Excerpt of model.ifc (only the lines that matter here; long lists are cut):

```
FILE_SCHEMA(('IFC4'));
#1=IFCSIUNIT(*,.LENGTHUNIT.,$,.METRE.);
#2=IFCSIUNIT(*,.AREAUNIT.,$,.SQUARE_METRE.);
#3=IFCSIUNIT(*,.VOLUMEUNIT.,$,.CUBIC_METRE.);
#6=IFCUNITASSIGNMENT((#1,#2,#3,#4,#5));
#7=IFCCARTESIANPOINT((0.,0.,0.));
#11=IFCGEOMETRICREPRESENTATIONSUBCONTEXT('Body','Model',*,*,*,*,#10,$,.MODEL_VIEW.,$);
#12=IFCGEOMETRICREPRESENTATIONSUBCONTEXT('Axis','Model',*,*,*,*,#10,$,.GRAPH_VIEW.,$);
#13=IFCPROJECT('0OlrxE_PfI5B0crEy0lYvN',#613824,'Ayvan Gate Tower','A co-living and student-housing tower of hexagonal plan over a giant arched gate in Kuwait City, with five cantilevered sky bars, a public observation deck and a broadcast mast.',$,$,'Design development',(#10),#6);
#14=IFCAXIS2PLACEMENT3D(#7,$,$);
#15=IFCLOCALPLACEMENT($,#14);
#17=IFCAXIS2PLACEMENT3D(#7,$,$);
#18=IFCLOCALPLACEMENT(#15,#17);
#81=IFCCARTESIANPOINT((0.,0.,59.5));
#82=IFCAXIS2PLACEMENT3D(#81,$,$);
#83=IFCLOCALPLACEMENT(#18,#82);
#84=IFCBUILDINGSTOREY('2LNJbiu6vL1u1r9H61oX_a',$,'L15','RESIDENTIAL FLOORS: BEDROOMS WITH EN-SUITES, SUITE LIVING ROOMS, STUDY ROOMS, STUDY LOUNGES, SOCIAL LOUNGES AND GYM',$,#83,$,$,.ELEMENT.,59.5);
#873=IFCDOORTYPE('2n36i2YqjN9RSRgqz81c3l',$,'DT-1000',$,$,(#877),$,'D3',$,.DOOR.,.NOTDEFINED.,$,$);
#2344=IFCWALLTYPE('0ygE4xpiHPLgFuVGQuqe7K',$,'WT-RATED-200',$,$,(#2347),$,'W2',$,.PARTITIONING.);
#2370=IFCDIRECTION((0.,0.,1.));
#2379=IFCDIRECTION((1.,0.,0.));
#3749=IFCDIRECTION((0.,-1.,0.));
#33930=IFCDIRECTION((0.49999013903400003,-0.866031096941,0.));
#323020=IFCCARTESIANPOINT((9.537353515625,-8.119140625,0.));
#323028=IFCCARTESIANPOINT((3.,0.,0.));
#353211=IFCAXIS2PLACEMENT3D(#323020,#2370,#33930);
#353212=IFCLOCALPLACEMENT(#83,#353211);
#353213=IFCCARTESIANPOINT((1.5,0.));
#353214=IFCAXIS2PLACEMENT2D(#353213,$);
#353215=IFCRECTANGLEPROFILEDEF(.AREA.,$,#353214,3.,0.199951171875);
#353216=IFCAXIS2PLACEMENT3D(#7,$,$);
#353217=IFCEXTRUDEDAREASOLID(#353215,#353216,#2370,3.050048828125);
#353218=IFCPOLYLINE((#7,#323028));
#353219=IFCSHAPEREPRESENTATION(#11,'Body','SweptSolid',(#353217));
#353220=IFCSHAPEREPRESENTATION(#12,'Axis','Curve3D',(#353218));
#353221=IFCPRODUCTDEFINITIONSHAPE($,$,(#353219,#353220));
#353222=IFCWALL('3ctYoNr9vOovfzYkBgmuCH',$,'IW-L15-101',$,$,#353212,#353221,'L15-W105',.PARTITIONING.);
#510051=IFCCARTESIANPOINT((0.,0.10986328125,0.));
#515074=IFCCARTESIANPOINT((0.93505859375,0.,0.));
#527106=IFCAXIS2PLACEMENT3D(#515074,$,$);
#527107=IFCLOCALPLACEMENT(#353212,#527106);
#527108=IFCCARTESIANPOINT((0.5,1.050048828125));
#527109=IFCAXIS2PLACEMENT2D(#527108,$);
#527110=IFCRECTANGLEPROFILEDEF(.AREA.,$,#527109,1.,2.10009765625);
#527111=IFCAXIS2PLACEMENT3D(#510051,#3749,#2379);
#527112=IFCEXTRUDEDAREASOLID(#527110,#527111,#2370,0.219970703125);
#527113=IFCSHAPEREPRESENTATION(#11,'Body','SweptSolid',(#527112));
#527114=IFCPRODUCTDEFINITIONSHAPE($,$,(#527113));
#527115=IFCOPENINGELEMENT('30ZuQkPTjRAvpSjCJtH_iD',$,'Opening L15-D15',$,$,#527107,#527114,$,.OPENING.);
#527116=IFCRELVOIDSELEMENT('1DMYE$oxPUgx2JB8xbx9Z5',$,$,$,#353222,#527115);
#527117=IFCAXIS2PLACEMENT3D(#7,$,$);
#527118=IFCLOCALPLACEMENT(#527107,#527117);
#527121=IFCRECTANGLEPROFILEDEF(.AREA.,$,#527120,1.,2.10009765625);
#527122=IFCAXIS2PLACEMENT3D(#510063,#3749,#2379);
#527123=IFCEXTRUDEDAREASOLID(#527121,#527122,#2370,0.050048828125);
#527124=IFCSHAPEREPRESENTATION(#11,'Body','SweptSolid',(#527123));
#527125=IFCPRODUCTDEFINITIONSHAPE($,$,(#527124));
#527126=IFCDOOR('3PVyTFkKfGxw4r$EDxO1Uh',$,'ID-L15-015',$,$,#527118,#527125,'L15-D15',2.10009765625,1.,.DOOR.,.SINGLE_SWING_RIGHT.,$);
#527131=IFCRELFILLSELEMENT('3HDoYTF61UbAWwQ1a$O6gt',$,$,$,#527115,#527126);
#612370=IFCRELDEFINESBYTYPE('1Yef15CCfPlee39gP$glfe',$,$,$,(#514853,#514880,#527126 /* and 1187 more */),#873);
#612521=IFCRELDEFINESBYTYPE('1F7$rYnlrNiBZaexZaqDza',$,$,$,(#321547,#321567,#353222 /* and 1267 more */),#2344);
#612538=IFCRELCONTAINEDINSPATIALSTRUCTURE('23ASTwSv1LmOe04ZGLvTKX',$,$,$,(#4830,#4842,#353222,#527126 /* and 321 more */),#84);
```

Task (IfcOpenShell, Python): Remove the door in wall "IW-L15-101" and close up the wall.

```python
import ifcopenshell
import ifcopenshell.api.feature
import ifcopenshell.api.root
import ifcopenshell.geom
import ifcopenshell.util.shape

model = ifcopenshell.open("model.ifc")
settings = ifcopenshell.geom.settings()


def volume(element):
    """Net volume in cubic metres, openings subtracted."""
    shape = ifcopenshell.geom.create_shape(settings, element)
    return ifcopenshell.util.shape.get_volume(shape.geometry)


door = model.by_guid("3PVyTFkKfGxw4r$EDxO1Uh")
opening = door.FillsVoids[0].RelatingOpeningElement
wall = opening.VoidsElements[0].RelatingBuildingElement
before = volume(wall)

ifcopenshell.api.root.remove_product(model, product=door)
ifcopenshell.api.feature.remove_feature(model, feature=opening)

after = volume(wall)

print(f"wall volume {before:.3f} -> {after:.3f} m3")

model.write("model_edited.ifc")
```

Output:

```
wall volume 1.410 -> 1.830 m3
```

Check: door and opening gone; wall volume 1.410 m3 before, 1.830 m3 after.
